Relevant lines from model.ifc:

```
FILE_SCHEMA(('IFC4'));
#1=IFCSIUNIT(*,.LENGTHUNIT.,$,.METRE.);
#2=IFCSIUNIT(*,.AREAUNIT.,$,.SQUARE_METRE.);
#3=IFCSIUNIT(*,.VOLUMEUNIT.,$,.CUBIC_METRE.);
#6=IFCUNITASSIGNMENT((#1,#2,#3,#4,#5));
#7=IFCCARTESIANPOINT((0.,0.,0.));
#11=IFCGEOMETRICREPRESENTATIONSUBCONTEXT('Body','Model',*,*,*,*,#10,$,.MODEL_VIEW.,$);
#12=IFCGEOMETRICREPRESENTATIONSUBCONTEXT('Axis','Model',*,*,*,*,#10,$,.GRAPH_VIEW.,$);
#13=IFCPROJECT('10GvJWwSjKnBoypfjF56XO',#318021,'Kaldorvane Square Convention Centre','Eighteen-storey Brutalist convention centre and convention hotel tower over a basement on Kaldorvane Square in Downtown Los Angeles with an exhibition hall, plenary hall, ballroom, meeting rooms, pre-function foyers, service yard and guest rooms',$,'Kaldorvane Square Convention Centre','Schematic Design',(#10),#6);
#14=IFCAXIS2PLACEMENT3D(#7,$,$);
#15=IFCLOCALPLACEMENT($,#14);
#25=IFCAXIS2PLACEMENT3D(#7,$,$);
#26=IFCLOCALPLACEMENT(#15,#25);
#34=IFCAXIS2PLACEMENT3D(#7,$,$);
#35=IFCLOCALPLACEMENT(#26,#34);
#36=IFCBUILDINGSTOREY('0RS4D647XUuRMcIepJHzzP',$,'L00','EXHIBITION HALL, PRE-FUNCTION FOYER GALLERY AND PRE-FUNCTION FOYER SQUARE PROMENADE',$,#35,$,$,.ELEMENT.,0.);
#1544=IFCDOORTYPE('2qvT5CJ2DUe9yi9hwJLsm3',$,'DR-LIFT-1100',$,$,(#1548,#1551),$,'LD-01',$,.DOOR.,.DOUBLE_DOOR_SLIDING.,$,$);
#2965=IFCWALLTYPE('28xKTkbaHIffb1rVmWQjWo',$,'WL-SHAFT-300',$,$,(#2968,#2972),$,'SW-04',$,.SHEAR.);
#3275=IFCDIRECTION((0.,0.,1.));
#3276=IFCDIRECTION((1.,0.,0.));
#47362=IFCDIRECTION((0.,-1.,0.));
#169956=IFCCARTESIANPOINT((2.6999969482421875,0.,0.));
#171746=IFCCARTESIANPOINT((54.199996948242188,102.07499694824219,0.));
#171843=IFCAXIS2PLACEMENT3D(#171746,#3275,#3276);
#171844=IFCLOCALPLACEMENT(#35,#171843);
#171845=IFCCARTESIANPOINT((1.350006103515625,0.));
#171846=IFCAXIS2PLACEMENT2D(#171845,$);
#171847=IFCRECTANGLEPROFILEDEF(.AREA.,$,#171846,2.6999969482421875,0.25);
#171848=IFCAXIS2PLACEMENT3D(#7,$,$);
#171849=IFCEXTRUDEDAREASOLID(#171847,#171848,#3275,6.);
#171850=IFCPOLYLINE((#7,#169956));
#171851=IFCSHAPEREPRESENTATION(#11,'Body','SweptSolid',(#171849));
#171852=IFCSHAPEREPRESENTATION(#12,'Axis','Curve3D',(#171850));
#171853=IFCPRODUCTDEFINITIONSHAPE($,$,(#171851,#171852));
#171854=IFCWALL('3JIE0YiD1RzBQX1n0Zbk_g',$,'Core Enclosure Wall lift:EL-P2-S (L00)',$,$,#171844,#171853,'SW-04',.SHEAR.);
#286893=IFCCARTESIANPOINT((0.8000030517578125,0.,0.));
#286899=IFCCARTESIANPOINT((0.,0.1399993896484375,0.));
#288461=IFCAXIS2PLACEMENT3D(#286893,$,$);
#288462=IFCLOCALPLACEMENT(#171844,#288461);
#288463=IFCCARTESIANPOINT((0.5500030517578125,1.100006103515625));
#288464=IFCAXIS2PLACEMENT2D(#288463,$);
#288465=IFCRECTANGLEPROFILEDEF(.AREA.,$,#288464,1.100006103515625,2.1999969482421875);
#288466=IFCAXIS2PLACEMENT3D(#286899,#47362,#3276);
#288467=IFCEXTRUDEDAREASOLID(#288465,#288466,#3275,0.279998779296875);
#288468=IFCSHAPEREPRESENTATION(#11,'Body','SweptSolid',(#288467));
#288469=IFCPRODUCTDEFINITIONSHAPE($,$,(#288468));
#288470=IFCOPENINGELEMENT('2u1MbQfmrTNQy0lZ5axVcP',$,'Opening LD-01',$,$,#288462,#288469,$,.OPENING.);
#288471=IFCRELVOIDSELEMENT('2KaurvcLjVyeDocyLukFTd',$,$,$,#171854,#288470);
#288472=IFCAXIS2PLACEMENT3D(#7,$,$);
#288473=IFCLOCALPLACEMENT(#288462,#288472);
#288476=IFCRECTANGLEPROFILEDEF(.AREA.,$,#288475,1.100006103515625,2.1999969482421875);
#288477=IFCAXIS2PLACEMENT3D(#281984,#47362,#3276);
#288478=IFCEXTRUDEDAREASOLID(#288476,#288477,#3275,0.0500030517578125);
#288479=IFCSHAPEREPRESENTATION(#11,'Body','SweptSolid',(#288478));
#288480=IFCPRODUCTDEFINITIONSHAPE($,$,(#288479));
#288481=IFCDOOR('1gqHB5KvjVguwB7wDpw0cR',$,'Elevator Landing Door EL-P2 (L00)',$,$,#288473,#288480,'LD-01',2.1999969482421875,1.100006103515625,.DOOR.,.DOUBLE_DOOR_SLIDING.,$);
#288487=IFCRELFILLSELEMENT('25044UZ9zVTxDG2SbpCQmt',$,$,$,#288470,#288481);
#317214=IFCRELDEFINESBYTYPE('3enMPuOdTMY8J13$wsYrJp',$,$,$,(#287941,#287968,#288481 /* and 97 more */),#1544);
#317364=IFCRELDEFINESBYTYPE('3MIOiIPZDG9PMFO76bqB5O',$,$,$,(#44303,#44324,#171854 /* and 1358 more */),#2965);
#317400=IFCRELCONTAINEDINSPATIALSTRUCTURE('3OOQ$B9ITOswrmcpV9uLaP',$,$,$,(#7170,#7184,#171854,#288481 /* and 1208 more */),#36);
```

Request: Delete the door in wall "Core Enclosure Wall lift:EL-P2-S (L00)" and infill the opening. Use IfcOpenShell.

```python
import ifcopenshell
import ifcopenshell.api.feature
import ifcopenshell.api.root
import ifcopenshell.geom
import ifcopenshell.util.shape

model = ifcopenshell.open("model.ifc")
settings = ifcopenshell.geom.settings()


def volume(element):
    """Net volume in cubic metres, openings subtracted."""
    shape = ifcopenshell.geom.create_shape(settings, element)
    return ifcopenshell.util.shape.get_volume(shape.geometry)


door = model.by_guid("1gqHB5KvjVguwB7wDpw0cR")
opening = door.FillsVoids[0].RelatingOpeningElement
wall = opening.VoidsElements[0].RelatingBuildingElement
before = volume(wall)

ifcopenshell.api.root.remove_product(model, product=door)
ifcopenshell.api.feature.remove_feature(model, feature=opening)

after = volume(wall)

print(f"wall volume {before:.3f} -> {after:.3f} m3")

model.write("model-out.ifc")
```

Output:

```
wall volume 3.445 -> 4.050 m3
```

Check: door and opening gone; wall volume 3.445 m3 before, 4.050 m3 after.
